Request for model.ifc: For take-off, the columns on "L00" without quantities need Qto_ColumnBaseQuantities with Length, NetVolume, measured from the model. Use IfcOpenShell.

First a look at what the model holds.

```python
import ifcopenshell
import ifcopenshell.util.element
import ifcopenshell.util.unit

model = ifcopenshell.open("model.ifc")
print(model.schema)
for unit_type in ("LENGTHUNIT", "AREAUNIT", "VOLUMEUNIT"):
    print(unit_type, ifcopenshell.util.unit.calculate_unit_scale(model, unit_type))
storey = next(s for s in model.by_type("IfcBuildingStorey") if s.Name == "L00")
columns = [e for e in ifcopenshell.util.element.get_decomposition(storey) if e.is_a("IfcColumn")]
for e in sorted(columns, key=lambda e: e.id()):
    print(e.id(), e.is_a(), e.Name, list(ifcopenshell.util.element.get_psets(e, qtos_only=True)), sep=" | ")
```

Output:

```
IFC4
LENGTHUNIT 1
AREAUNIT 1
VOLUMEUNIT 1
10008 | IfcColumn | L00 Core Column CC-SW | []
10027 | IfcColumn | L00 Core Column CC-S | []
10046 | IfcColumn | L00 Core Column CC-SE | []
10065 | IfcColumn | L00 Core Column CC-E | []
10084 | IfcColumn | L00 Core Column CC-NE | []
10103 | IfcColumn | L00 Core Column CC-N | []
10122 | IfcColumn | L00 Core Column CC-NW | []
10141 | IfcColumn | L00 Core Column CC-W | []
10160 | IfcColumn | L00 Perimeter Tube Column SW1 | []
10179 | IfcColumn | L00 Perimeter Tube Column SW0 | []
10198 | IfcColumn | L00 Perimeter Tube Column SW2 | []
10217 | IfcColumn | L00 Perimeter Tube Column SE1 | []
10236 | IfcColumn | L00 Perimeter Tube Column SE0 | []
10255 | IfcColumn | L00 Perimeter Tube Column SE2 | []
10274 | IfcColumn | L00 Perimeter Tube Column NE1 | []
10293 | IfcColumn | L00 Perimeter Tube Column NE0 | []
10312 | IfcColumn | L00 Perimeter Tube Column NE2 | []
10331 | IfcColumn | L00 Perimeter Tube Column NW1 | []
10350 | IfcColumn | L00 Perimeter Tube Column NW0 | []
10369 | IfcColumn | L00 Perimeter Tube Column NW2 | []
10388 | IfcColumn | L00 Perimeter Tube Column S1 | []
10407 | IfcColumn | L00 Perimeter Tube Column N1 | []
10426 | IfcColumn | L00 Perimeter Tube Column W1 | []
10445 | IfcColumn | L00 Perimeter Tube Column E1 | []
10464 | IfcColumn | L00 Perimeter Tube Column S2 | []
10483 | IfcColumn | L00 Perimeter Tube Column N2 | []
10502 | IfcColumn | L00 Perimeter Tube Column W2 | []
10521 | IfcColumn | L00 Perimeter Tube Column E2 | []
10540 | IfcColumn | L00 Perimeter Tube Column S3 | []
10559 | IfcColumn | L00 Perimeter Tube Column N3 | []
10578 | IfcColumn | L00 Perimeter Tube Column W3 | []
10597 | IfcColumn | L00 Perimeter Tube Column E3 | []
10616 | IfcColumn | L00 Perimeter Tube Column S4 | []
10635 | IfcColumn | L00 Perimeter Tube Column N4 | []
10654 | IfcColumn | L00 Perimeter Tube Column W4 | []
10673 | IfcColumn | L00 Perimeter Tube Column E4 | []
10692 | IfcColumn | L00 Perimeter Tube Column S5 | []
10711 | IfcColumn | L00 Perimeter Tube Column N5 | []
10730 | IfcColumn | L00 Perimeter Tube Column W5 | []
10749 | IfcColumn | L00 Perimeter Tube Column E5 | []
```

```python
import ifcopenshell
import ifcopenshell.api.pset
import ifcopenshell.geom
import ifcopenshell.util.element
import ifcopenshell.util.shape
import ifcopenshell.util.unit

model = ifcopenshell.open("model.ifc")
unit_scale = ifcopenshell.util.unit.calculate_unit_scale(model)
volume_scale = ifcopenshell.util.unit.calculate_unit_scale(model, "VOLUMEUNIT")
settings = ifcopenshell.geom.settings()

storey = next(s for s in model.by_type("IfcBuildingStorey") if s.Name == "L00")
columns = [e for e in ifcopenshell.util.element.get_decomposition(storey) if e.is_a("IfcColumn")]

for e in sorted(columns, key=lambda e: e.id()):
    if ifcopenshell.util.element.get_psets(e, qtos_only=True, should_inherit=False):
        continue
    # Geometry comes back in metres, in the element's own axes.
    shape = ifcopenshell.geom.create_shape(settings, e)
    values = {
        "Length": ifcopenshell.util.shape.get_z(shape.geometry) / unit_scale,
        "NetVolume": ifcopenshell.util.shape.get_volume(shape.geometry) / volume_scale,
    }
    qto = ifcopenshell.api.pset.add_qto(model, product=e, name="Qto_ColumnBaseQuantities")
    ifcopenshell.api.pset.edit_qto(model, qto=qto, properties=values)
    print(e.id(), {k: round(v, 3) for k, v in values.items()})

model.write("model_v2.ifc")
```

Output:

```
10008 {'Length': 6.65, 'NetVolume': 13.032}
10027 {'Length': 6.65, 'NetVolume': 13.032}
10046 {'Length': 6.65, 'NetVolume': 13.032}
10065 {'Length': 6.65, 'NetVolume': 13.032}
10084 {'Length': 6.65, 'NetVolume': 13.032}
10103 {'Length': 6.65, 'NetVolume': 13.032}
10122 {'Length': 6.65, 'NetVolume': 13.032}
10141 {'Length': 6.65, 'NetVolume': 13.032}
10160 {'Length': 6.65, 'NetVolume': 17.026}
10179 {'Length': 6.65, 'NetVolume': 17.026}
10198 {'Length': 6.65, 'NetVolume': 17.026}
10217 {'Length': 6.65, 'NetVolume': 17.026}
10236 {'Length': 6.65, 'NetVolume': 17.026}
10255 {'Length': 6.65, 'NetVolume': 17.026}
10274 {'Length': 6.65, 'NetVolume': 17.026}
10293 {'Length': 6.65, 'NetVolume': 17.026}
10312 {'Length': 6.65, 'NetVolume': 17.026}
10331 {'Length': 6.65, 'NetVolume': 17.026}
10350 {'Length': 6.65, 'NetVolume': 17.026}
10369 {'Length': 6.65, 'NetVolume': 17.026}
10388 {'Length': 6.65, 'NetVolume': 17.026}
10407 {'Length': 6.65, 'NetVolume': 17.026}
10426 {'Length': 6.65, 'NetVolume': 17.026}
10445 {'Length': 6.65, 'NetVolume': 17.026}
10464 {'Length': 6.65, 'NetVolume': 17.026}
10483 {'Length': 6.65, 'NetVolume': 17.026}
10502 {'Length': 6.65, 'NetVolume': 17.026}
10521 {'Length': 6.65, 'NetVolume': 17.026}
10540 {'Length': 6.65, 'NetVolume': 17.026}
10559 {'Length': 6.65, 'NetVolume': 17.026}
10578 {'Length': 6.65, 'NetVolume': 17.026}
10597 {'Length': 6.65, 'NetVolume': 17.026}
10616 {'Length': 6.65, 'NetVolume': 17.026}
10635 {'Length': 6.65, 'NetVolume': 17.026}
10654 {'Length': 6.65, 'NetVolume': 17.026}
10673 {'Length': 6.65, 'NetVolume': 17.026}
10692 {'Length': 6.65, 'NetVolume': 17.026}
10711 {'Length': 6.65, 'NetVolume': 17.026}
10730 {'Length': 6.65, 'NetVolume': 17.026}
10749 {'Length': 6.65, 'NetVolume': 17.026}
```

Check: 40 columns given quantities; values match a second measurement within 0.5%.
